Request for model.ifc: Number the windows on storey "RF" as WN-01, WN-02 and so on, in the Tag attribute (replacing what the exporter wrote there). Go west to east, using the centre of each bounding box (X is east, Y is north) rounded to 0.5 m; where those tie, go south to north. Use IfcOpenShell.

First a look at what the model holds.

```python
import ifcopenshell
import ifcopenshell.util.element
import ifcopenshell.util.placement

model = ifcopenshell.open("model.ifc")
print(model.schema)
storey = next(s for s in model.by_type("IfcBuildingStorey") if s.Name == "RF")
windows = [e for e in ifcopenshell.util.element.get_decomposition(storey) if e.is_a("IfcWindow")]
for e in sorted(windows, key=lambda e: e.id()):
    origin = ifcopenshell.util.placement.get_local_placement(e.ObjectPlacement)[:3, 3]
    print(e.id(), e.Tag, e.Name, origin.round(2) + 0.0, sep=" | ")
```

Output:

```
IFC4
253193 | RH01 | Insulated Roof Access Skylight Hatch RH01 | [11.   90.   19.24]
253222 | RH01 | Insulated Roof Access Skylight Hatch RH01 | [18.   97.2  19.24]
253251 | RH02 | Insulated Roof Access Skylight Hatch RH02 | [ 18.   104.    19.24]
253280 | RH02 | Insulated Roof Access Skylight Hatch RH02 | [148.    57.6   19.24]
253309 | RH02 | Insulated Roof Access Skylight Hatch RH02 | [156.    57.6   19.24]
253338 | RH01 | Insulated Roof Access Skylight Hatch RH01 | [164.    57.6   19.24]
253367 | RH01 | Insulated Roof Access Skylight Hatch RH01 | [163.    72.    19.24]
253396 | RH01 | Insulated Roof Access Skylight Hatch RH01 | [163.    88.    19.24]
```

```python
import ifcopenshell
import ifcopenshell.geom
import ifcopenshell.util.element
import ifcopenshell.util.shape

model = ifcopenshell.open("model.ifc")
settings = ifcopenshell.geom.settings()
settings.set("use-world-coords", True)


def centre(element):
    shape = ifcopenshell.geom.create_shape(settings, element)
    return ifcopenshell.util.shape.get_bbox_centroid(shape.geometry)


storey = next(s for s in model.by_type("IfcBuildingStorey") if s.Name == "RF")
windows = [e for e in ifcopenshell.util.element.get_decomposition(storey) if e.is_a("IfcWindow")]

# Insertion points can sit at a corner or the storey origin, so sort by the geometry (in metres).
centres = {e: centre(e) for e in windows}
windows.sort(key=lambda e: (round(centres[e][0] / 0.5), centres[e][1]))

for i, e in enumerate(windows, start=1):
    number = f"WN-{i:02d}"
    e.Tag = number
    print(e.id(), number)

model.write("model_v2.ifc")
```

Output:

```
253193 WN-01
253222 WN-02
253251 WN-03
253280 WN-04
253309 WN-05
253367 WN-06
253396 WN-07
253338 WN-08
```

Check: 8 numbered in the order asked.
